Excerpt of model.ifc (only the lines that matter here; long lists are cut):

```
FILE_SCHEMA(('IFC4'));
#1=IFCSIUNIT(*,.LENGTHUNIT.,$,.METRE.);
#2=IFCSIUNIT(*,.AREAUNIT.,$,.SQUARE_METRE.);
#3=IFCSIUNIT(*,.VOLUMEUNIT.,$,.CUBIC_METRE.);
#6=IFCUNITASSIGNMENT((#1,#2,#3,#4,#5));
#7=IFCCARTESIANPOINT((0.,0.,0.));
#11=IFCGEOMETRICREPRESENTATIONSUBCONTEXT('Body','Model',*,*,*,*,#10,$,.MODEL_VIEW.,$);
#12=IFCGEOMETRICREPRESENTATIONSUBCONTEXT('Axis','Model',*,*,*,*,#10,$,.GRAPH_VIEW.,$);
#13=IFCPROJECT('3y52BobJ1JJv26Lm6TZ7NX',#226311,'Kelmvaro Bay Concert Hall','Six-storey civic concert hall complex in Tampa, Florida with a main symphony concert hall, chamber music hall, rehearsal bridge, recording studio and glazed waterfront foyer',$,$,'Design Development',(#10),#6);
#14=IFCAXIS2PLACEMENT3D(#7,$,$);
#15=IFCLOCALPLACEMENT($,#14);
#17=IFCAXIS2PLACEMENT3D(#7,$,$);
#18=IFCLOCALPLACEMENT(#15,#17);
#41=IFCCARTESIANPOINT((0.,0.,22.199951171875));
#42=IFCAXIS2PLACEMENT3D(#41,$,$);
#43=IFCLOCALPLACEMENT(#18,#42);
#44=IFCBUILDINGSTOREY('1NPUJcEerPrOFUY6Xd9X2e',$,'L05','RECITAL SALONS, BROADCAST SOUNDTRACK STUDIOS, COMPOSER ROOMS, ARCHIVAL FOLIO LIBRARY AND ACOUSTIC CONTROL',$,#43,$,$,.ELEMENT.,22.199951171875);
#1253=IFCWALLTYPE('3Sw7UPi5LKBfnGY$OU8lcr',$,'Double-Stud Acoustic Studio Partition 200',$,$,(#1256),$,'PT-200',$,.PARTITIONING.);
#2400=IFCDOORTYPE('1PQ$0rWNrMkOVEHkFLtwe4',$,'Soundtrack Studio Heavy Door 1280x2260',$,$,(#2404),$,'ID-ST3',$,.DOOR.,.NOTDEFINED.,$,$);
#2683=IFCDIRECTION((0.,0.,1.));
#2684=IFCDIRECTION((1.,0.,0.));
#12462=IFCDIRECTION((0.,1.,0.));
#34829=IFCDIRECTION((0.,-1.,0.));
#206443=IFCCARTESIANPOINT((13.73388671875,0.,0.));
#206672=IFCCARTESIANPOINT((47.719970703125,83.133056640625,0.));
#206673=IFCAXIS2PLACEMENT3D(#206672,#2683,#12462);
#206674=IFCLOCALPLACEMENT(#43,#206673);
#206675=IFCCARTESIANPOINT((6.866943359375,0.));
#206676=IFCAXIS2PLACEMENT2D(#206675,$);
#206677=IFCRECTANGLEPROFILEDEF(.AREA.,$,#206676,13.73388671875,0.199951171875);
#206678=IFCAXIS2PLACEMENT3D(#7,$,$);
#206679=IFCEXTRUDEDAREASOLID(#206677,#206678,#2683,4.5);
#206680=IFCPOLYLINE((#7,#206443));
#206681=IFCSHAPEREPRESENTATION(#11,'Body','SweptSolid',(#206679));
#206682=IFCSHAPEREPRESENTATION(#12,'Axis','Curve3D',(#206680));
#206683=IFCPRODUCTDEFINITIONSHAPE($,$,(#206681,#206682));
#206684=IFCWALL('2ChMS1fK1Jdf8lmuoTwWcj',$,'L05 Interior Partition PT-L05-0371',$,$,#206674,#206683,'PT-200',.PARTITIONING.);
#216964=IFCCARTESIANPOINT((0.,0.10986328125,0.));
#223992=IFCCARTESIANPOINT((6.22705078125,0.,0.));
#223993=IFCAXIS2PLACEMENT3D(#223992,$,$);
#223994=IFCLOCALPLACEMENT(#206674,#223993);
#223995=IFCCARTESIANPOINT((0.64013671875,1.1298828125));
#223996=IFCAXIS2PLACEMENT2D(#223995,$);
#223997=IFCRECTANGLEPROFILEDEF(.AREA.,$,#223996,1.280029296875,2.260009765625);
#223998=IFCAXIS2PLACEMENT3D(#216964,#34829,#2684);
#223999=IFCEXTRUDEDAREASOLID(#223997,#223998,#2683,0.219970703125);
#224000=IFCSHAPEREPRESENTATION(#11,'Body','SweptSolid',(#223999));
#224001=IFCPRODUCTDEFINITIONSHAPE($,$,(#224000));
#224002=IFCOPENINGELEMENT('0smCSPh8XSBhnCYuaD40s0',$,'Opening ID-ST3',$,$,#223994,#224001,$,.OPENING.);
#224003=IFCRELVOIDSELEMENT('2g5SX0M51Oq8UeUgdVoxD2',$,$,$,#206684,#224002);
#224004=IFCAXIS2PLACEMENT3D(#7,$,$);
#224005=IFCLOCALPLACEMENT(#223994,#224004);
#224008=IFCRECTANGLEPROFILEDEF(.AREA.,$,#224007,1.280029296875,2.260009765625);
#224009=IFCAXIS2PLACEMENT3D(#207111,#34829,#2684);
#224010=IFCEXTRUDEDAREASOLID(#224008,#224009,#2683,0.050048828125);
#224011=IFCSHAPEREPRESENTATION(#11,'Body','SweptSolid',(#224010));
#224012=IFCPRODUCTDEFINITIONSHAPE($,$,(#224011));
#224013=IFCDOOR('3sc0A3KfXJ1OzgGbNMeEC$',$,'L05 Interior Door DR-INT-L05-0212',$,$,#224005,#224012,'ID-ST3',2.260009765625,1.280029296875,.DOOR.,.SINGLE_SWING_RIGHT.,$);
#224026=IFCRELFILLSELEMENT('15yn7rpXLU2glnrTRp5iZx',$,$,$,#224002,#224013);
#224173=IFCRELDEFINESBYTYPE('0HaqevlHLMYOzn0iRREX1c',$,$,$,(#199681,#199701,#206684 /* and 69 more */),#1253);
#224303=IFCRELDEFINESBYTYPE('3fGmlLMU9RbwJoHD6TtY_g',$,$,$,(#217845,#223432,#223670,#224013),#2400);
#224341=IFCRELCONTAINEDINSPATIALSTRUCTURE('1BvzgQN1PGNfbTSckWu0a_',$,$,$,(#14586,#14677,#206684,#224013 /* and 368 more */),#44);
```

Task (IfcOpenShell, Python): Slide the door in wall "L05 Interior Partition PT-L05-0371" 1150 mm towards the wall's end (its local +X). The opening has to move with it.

```python
import ifcopenshell
import ifcopenshell.api.geometry
import ifcopenshell.util.placement

model = ifcopenshell.open("model.ifc")

door = model.by_id(224013)
opening = door.FillsVoids[0].RelatingOpeningElement
wall = opening.VoidsElements[0].RelatingBuildingElement

wall_matrix = ifcopenshell.util.placement.get_local_placement(wall.ObjectPlacement)
shift = wall_matrix[:3, 0] * 1.15
before = ifcopenshell.util.placement.get_local_placement(door.ObjectPlacement)[:3, 3].copy()

# The door is placed relative to its opening, so it follows when the opening moves.
matrix = ifcopenshell.util.placement.get_local_placement(opening.ObjectPlacement)
matrix[:3, 3] += shift
ifcopenshell.api.geometry.edit_object_placement(
    model, product=opening, matrix=matrix, is_si=False, should_transform_children=True
)

after = ifcopenshell.util.placement.get_local_placement(door.ObjectPlacement)[:3, 3]
print("door moved by", (after - before).round(3) + 0.0)

model.write("model_v2.ifc")
```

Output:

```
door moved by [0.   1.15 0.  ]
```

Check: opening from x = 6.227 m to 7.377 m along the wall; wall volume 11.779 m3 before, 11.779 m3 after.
